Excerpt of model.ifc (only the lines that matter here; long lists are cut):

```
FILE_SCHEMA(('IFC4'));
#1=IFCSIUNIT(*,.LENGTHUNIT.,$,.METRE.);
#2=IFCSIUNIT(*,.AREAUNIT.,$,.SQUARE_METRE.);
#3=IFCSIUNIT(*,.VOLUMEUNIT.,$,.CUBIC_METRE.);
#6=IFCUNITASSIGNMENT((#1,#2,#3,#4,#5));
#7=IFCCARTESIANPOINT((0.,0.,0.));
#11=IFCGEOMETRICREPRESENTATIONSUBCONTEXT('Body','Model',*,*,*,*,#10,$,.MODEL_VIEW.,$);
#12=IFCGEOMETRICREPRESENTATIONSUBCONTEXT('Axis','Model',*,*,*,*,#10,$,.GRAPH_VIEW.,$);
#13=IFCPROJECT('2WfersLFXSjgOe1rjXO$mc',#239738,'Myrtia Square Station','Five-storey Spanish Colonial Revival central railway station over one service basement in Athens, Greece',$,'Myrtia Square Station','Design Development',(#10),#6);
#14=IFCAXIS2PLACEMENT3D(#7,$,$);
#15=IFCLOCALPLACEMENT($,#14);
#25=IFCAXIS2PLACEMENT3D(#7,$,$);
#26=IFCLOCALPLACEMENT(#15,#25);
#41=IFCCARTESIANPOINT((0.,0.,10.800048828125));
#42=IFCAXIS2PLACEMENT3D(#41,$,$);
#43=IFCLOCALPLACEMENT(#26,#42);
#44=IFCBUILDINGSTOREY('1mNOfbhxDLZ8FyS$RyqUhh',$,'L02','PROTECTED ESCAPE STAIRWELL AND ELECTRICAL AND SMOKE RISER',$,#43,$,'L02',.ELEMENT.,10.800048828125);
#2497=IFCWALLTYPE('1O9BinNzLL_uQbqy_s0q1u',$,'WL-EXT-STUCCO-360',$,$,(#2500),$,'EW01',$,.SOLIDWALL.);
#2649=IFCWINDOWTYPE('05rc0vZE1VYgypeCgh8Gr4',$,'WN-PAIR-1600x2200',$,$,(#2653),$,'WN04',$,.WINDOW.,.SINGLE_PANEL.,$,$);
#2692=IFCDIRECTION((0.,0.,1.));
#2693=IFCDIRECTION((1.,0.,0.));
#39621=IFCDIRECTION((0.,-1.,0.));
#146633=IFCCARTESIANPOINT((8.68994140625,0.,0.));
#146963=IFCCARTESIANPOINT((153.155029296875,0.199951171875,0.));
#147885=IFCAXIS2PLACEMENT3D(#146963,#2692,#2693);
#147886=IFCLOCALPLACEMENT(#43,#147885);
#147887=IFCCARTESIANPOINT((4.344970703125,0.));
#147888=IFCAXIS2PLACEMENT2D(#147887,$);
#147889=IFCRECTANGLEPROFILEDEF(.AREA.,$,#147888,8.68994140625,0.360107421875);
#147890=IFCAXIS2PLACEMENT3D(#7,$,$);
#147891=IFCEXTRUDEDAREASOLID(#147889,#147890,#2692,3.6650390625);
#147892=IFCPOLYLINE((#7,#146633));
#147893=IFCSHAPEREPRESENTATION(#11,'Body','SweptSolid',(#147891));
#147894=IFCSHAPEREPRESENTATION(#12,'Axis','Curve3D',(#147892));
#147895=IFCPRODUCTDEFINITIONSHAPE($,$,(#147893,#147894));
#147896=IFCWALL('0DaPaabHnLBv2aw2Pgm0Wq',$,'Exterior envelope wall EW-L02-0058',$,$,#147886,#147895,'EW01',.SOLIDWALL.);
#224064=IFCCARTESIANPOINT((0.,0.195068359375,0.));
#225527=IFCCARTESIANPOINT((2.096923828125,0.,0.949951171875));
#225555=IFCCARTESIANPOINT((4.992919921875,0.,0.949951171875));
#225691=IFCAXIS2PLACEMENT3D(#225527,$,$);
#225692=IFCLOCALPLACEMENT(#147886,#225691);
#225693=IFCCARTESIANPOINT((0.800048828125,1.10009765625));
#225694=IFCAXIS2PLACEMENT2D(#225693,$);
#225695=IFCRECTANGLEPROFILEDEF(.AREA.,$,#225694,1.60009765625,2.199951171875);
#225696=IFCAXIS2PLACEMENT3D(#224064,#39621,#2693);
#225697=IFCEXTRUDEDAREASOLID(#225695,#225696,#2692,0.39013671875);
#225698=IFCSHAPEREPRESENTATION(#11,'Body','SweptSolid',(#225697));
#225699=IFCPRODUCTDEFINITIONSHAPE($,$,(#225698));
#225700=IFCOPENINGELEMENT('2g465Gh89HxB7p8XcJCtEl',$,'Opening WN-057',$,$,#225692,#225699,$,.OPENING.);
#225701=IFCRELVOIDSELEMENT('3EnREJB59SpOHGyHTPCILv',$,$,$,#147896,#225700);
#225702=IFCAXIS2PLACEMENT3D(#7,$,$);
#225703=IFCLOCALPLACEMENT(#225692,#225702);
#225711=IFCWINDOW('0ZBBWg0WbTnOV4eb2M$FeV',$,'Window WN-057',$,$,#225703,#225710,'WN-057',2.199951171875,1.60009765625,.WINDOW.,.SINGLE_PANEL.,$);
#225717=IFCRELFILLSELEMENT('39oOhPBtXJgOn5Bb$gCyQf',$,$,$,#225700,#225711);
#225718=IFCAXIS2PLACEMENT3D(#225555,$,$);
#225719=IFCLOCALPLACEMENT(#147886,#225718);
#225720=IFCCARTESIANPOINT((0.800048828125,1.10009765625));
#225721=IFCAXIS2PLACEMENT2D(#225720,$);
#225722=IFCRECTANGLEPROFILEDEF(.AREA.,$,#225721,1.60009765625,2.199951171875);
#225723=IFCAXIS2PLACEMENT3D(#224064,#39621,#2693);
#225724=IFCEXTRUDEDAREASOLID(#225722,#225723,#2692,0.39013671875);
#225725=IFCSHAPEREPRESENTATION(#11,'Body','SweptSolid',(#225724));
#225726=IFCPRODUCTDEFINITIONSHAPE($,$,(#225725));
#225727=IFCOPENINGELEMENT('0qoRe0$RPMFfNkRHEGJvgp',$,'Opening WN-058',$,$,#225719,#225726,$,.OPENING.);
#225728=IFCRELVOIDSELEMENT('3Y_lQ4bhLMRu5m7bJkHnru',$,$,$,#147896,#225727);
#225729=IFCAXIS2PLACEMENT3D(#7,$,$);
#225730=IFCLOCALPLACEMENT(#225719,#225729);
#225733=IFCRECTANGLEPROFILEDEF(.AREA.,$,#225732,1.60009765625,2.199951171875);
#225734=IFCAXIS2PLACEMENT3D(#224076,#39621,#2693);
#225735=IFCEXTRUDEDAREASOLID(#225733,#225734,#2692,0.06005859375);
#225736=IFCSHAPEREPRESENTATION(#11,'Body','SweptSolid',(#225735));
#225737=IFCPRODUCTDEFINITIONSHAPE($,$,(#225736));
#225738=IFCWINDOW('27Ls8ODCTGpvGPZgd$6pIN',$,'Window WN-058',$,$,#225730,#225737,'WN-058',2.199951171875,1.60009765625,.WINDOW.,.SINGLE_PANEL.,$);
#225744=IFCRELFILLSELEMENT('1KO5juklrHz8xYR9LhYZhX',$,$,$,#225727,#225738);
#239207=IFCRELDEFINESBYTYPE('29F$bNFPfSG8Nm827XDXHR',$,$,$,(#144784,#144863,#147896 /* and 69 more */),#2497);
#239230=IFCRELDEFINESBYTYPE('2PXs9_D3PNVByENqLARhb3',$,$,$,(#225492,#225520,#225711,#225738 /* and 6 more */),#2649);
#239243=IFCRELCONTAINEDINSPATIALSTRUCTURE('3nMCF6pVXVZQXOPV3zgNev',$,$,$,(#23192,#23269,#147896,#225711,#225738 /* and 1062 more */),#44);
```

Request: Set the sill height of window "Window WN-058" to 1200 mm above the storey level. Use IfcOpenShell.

```python
import numpy as np
import ifcopenshell
import ifcopenshell.api.geometry
import ifcopenshell.geom
import ifcopenshell.util.element
import ifcopenshell.util.placement
import ifcopenshell.util.shape
import ifcopenshell.util.unit

model = ifcopenshell.open("model.ifc")
unit_scale = ifcopenshell.util.unit.calculate_unit_scale(model)

window = model.by_guid("27Ls8ODCTGpvGPZgd$6pIN")
opening = window.FillsVoids[0].RelatingOpeningElement
storey = ifcopenshell.util.element.get_container(window, ifc_class="IfcBuildingStorey")
level = ifcopenshell.util.placement.get_local_placement(storey.ObjectPlacement)[2, 3]

# The opening's origin need not be at the sill, so measure its lowest point.
shape = ifcopenshell.geom.create_shape(ifcopenshell.geom.settings(), opening)
bottom = ifcopenshell.util.shape.get_shape_bottom_elevation(shape, shape.geometry) / unit_scale
dz = level + 1.2 - bottom

shift = np.array([0.0, 0.0, dz])
# The window is placed relative to its opening, so it follows when the opening moves.
matrix = ifcopenshell.util.placement.get_local_placement(opening.ObjectPlacement)
matrix[:3, 3] += shift
ifcopenshell.api.geometry.edit_object_placement(
    model, product=opening, matrix=matrix, is_si=False, should_transform_children=True
)

print(f"moved by {dz * unit_scale:+.3f} m")

model.write("model_updated.ifc")
```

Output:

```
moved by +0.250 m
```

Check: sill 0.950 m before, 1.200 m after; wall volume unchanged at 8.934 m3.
